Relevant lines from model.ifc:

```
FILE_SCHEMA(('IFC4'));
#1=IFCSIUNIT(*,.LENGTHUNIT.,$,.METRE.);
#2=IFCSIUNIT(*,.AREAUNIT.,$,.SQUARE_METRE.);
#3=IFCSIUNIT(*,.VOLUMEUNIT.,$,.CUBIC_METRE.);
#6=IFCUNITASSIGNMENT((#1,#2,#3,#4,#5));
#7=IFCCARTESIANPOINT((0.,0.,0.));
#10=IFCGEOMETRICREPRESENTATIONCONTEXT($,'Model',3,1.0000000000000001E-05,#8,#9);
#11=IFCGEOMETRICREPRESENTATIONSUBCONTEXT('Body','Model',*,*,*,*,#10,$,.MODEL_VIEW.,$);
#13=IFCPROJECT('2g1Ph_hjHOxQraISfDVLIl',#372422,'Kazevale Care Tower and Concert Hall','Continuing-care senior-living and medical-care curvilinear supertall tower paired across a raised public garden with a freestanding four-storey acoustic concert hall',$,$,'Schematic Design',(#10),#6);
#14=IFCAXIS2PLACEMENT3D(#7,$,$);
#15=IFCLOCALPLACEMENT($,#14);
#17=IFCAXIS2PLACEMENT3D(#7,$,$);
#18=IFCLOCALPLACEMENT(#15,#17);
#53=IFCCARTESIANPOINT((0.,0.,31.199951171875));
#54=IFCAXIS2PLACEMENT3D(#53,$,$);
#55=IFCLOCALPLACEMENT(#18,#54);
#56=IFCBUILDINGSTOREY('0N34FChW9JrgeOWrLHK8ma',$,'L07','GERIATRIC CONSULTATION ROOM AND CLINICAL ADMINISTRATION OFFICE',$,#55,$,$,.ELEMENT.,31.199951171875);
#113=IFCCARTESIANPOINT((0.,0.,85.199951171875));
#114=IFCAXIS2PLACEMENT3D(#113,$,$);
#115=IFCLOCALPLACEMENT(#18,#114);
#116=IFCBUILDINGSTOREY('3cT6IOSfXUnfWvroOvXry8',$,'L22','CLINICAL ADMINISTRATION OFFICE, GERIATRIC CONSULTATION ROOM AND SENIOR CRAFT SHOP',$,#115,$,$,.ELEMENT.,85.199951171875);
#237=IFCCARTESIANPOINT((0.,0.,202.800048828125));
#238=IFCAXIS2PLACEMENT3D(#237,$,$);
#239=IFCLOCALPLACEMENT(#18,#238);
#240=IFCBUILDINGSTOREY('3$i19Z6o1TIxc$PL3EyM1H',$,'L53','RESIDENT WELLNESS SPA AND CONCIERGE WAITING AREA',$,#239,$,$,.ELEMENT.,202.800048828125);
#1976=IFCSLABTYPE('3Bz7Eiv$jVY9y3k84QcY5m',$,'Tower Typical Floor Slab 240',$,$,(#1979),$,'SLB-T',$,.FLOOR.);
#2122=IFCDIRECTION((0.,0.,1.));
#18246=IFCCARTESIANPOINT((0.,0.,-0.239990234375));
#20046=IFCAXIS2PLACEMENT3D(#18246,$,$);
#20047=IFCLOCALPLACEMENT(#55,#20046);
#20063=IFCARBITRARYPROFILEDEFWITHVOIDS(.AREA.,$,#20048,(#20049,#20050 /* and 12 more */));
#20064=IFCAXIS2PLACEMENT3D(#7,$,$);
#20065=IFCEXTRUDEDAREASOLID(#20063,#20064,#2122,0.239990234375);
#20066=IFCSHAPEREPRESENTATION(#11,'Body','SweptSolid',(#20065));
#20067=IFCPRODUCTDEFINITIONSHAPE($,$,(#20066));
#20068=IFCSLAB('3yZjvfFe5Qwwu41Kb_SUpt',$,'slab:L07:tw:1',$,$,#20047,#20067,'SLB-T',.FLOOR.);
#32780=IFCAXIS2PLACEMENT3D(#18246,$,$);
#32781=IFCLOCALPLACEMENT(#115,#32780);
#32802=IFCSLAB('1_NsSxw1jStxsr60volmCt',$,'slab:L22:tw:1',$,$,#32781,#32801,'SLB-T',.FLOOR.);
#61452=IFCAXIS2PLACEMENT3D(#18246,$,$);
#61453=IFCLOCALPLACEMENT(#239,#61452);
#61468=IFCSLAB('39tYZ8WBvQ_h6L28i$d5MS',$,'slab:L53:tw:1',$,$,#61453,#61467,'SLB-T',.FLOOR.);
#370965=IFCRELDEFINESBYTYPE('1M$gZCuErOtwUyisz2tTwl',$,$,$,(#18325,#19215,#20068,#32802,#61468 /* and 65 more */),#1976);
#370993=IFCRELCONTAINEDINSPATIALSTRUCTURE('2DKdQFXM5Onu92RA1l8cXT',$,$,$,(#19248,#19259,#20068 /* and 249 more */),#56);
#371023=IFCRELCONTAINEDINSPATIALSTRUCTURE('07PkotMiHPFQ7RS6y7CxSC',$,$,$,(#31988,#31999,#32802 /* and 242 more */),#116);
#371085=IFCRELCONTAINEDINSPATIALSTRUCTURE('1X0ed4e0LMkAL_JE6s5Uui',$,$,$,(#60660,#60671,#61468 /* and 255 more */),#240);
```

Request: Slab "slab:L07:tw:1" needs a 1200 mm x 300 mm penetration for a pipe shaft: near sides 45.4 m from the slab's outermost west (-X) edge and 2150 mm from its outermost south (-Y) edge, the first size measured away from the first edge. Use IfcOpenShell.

```python
import numpy as np
import ifcopenshell
import ifcopenshell.api.feature
import ifcopenshell.api.geometry
import ifcopenshell.api.root
import ifcopenshell.geom
import ifcopenshell.util.placement
import ifcopenshell.util.representation
import ifcopenshell.util.shape
import ifcopenshell.util.unit

model = ifcopenshell.open("model.ifc")
unit_scale = ifcopenshell.util.unit.calculate_unit_scale(model)
settings = ifcopenshell.geom.settings()


def volume(element):
    """Net volume in cubic metres, openings subtracted."""
    shape = ifcopenshell.geom.create_shape(settings, element)
    return ifcopenshell.util.shape.get_volume(shape.geometry)


slab = model.by_id(20068)
before = volume(slab)

# Extent in the slab's own axes, in metres. The edges named are its -X and -Y sides.
slab_shape = ifcopenshell.geom.create_shape(settings, slab)
vertices = ifcopenshell.util.shape.get_vertices(slab_shape.geometry)
x_min, y_min, bottom = vertices.min(axis=0)
top = vertices[:, 2].max()

opening = ifcopenshell.api.root.create_entity(model, ifc_class="IfcOpeningElement", name="Pipe shaft opening", predefined_type="OPENING")
context = ifcopenshell.util.representation.get_context(model, "Model", "Body", "MODEL_VIEW")
width, depth = 1.2, 0.3
outline = [(0.0, 0.0), (width, 0.0), (width, depth), (0.0, depth), (0.0, 0.0)]
# Overshoot both faces by 50 mm so the cut is clean.
shape = ifcopenshell.api.geometry.add_slab_representation(
    model, context=context, depth=top - bottom + 0.1, polyline=outline
)
ifcopenshell.api.geometry.assign_representation(model, product=opening, representation=shape)

matrix = ifcopenshell.util.placement.get_local_placement(slab.ObjectPlacement)
matrix[:, 3] = matrix @ np.append(np.array([x_min + 45.4, y_min + 2.15, bottom - 0.05]) / unit_scale, 1.0)
ifcopenshell.api.geometry.edit_object_placement(model, product=opening, matrix=matrix, is_si=False)
ifcopenshell.api.feature.add_feature(model, feature=opening, element=slab)

after = volume(slab)

print(f"slab volume {before:.3f} -> {after:.3f} m3")

model.write("model-out.ifc")
```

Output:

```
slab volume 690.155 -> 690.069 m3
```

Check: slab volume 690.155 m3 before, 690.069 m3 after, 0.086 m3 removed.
